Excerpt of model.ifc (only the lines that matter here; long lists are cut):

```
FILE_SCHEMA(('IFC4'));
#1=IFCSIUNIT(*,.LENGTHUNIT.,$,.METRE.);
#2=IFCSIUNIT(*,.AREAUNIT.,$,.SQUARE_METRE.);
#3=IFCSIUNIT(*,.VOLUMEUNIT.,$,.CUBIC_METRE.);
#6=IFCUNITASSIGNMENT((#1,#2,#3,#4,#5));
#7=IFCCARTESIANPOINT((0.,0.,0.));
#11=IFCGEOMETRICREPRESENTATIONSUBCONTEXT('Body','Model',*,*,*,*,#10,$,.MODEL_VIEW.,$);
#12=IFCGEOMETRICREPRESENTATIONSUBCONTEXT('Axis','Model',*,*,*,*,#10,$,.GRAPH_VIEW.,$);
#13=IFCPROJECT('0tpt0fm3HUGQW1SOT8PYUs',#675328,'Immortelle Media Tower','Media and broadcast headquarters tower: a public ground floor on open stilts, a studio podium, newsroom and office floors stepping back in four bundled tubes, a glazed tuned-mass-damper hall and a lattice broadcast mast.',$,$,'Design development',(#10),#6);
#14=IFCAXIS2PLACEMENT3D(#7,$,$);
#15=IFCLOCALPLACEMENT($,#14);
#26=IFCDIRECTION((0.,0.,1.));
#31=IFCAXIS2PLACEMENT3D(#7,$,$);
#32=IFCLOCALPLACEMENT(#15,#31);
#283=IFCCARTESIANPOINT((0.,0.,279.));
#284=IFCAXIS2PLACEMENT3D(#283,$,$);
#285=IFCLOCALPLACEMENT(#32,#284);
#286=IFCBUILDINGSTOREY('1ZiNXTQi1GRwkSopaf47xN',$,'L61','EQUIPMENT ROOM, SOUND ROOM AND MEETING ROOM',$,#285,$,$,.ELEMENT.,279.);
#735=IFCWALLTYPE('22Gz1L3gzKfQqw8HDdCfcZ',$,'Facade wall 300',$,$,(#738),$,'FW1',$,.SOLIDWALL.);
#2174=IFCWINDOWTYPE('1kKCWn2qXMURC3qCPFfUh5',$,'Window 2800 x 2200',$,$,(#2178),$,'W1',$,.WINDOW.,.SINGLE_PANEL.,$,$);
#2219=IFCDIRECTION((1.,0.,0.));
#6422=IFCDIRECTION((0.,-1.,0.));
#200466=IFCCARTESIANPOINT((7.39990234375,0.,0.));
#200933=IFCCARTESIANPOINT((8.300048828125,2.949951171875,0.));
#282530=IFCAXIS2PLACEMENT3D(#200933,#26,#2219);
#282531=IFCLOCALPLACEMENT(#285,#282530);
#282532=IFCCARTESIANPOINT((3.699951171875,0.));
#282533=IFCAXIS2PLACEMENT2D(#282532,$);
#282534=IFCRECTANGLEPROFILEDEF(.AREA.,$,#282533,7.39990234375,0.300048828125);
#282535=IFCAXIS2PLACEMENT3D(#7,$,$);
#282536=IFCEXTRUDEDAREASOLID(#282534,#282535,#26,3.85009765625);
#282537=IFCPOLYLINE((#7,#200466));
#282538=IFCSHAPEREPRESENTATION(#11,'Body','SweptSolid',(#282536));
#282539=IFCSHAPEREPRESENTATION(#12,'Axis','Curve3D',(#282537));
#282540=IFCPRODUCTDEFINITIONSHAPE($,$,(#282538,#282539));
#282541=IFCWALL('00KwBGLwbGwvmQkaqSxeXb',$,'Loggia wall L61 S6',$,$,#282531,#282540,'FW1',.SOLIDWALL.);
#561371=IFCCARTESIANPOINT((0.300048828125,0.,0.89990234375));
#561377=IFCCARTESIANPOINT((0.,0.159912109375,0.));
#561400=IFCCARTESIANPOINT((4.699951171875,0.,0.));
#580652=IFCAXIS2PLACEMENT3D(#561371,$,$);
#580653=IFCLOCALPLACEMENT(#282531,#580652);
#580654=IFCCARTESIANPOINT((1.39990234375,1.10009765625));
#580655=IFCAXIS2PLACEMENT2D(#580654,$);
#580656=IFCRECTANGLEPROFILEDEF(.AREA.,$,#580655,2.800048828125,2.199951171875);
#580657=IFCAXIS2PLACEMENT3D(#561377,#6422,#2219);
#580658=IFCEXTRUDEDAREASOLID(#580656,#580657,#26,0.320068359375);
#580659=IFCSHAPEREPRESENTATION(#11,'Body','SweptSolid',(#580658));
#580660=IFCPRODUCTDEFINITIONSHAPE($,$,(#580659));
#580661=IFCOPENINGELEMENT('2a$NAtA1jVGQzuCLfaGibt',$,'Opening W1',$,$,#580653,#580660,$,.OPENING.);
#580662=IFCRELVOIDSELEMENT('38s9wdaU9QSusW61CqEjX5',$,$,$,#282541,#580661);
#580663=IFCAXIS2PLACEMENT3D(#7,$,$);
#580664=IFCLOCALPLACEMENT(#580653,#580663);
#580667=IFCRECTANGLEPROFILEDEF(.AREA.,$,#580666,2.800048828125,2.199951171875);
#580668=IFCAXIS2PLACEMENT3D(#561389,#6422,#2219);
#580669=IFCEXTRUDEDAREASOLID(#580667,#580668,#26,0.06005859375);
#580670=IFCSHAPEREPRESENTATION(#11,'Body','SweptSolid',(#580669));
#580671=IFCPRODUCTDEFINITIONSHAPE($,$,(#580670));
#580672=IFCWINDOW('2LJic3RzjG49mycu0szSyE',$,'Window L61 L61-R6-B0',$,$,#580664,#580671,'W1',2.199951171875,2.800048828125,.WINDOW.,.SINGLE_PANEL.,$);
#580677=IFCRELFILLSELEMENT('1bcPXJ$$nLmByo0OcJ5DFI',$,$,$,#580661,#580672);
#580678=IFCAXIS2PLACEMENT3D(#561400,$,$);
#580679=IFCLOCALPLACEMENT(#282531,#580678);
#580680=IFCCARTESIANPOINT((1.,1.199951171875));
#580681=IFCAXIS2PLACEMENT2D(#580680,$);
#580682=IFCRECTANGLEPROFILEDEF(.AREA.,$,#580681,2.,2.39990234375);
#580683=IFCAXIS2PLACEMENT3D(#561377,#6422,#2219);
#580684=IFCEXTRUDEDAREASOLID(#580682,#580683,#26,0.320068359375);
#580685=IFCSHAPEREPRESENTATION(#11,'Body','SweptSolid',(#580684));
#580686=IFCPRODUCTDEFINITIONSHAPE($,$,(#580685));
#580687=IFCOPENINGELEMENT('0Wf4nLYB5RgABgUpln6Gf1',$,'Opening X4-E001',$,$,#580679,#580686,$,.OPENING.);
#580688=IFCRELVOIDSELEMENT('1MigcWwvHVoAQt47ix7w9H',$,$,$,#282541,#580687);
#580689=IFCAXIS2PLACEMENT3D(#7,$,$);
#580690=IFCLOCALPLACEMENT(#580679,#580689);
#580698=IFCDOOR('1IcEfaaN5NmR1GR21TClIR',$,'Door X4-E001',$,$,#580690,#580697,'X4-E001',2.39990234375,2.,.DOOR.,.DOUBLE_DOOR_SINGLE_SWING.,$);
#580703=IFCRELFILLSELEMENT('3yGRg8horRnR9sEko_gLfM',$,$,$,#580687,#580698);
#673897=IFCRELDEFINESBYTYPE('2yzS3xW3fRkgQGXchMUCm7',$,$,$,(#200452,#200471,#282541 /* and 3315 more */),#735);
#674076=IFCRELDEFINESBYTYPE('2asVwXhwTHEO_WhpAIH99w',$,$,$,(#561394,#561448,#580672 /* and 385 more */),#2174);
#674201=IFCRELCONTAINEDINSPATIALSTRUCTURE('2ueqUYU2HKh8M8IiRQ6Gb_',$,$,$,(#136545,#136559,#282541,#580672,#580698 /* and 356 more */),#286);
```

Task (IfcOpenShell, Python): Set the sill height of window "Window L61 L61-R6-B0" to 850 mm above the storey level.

```python
import numpy as np
import ifcopenshell
import ifcopenshell.api.geometry
import ifcopenshell.geom
import ifcopenshell.util.element
import ifcopenshell.util.placement
import ifcopenshell.util.shape
import ifcopenshell.util.unit

model = ifcopenshell.open("model.ifc")
unit_scale = ifcopenshell.util.unit.calculate_unit_scale(model)

window = model.by_id(580672)
opening = window.FillsVoids[0].RelatingOpeningElement
storey = ifcopenshell.util.element.get_container(window, ifc_class="IfcBuildingStorey")
level = ifcopenshell.util.placement.get_local_placement(storey.ObjectPlacement)[2, 3]

# The opening's origin need not be at the sill, so measure its lowest point.
shape = ifcopenshell.geom.create_shape(ifcopenshell.geom.settings(), opening)
bottom = ifcopenshell.util.shape.get_shape_bottom_elevation(shape, shape.geometry) / unit_scale
dz = level + 0.85 / unit_scale - bottom

shift = np.array([0.0, 0.0, dz])
# The window is placed relative to its opening, so it follows when the opening moves.
matrix = ifcopenshell.util.placement.get_local_placement(opening.ObjectPlacement)
matrix[:3, 3] += shift
ifcopenshell.api.geometry.edit_object_placement(
    model, product=opening, matrix=matrix, is_si=False, should_transform_children=True
)

print(f"moved by {dz * unit_scale:+.3f} m")

model.write("model_rev.ifc")
```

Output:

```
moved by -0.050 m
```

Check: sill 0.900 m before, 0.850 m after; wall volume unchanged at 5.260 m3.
